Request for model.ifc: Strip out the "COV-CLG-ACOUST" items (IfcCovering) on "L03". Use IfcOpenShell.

First a look at what the model holds.

```python
import ifcopenshell
import ifcopenshell.util.element

model = ifcopenshell.open("model.ifc")
print(model.schema)
storey = next(s for s in model.by_type("IfcBuildingStorey") if s.Name == "L03")
coverings = [e for e in ifcopenshell.util.element.get_decomposition(storey) if e.is_a("IfcCovering")]
seen = {}
for e in coverings:
    element_type = ifcopenshell.util.element.get_type(e)
    name = element_type.Name if element_type not in (None, e) else None
    seen[name] = seen.get(name, 0) + 1
for name, count in sorted(seen.items(), key=str):
    print(count, "x", name)
```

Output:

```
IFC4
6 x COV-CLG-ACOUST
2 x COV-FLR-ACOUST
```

```python
import ifcopenshell
import ifcopenshell.api.root
import ifcopenshell.util.element

model = ifcopenshell.open("model.ifc")

storey = next(s for s in model.by_type("IfcBuildingStorey") if s.Name == "L03")
coverings = [e for e in ifcopenshell.util.element.get_decomposition(storey) if e.is_a("IfcCovering")]
targets = [e for e in coverings if (t := ifcopenshell.util.element.get_type(e)) not in (None, e) and t.Name == "COV-CLG-ACOUST"]

for e in targets:
    ifcopenshell.api.root.remove_product(model, product=e)
print(len(targets), "removed")

model.write("model-out.ifc")
```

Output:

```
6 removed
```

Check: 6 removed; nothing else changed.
